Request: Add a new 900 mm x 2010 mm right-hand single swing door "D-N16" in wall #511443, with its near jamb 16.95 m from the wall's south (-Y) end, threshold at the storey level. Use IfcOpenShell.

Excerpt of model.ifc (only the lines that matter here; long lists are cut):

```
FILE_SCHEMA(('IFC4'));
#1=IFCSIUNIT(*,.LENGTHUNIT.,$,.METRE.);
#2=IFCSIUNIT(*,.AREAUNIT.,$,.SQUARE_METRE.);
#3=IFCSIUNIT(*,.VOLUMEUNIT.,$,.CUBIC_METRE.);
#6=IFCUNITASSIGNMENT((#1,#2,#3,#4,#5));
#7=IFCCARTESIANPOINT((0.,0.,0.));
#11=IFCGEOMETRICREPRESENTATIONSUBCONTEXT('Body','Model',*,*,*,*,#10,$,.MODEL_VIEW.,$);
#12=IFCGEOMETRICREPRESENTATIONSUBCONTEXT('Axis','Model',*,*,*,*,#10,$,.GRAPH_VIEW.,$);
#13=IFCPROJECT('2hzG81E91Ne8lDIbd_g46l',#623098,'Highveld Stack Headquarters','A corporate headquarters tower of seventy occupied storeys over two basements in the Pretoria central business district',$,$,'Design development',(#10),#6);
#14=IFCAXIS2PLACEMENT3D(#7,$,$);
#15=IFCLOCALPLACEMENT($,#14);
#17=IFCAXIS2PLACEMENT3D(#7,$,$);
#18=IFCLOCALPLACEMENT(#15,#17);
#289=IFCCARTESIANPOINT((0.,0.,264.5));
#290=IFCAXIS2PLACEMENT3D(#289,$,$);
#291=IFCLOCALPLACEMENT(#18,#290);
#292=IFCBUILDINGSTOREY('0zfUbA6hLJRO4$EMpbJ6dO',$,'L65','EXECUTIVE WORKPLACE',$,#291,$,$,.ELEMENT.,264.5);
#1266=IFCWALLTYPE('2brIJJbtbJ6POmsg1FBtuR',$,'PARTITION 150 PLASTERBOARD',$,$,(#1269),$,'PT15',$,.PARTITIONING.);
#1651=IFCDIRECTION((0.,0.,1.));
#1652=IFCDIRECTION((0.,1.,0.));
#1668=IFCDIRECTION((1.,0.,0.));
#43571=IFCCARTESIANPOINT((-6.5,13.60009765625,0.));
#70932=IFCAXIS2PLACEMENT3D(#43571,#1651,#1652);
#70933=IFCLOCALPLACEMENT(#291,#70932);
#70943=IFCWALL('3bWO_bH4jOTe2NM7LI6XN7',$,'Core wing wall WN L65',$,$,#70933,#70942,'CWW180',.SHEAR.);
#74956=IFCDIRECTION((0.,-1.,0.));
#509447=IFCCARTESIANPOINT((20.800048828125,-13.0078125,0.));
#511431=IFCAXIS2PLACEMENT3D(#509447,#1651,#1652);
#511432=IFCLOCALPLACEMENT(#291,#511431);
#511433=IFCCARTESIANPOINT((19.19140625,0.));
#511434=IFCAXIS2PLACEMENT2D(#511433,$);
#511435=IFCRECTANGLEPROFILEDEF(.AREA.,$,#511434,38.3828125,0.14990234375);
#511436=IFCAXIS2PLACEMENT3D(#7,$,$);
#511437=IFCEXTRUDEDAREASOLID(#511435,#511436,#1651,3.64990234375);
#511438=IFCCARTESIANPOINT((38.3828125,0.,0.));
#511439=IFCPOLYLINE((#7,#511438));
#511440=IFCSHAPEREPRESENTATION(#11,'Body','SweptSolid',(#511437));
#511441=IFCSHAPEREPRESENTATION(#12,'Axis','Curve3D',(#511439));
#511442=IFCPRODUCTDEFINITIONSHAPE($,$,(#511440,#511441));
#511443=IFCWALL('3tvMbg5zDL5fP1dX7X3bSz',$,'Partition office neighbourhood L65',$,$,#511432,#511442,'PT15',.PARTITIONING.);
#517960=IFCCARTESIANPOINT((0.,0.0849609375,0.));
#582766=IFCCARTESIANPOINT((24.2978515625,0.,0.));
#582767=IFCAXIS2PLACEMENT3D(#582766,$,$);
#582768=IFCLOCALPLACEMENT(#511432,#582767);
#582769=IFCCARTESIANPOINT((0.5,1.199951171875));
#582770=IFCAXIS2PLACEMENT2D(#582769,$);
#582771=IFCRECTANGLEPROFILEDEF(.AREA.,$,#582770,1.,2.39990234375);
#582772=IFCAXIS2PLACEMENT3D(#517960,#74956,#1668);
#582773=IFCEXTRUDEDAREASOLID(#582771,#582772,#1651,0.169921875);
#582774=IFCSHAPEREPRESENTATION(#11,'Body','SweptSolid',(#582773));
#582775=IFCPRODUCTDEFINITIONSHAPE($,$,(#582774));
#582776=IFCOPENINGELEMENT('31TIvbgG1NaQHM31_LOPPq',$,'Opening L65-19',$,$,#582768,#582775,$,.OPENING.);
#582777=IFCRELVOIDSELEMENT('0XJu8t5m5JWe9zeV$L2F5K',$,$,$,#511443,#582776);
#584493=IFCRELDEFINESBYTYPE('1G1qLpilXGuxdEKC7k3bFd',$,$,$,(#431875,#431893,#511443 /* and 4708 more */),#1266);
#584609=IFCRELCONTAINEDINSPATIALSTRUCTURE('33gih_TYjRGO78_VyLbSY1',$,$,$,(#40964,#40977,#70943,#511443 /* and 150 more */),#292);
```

```python
import numpy as np
import ifcopenshell
import ifcopenshell.api.feature
import ifcopenshell.api.geometry
import ifcopenshell.api.root
import ifcopenshell.api.spatial
import ifcopenshell.geom
import ifcopenshell.util.element
import ifcopenshell.util.placement
import ifcopenshell.util.representation
import ifcopenshell.util.shape
import ifcopenshell.util.unit

model = ifcopenshell.open("model.ifc")
unit_scale = ifcopenshell.util.unit.calculate_unit_scale(model)
settings = ifcopenshell.geom.settings()


def volume(element):
    """Net volume in cubic metres, openings subtracted."""
    shape = ifcopenshell.geom.create_shape(settings, element)
    return ifcopenshell.util.shape.get_volume(shape.geometry)


wall = model.by_guid("3tvMbg5zDL5fP1dX7X3bSz")
storey = ifcopenshell.util.element.get_container(wall, ifc_class="IfcBuildingStorey")
context = ifcopenshell.util.representation.get_context(model, "Model", "Body", "MODEL_VIEW")
before = volume(wall)

width, height, from_end, sill = 0.9, 2.01, 16.95, 0.0  # metres

# The wall runs along its own X axis, and the end named is its -X end.
wall_shape = ifcopenshell.geom.create_shape(settings, wall)
x, y, z = ifcopenshell.util.shape.get_vertices(wall_shape.geometry).T
start = x.min() + from_end
face, thickness = float(y.min()), float(y.max() - y.min())
wall_matrix = ifcopenshell.util.placement.get_local_placement(wall.ObjectPlacement)
level = ifcopenshell.util.placement.get_local_placement(storey.ObjectPlacement)[2, 3]


def in_wall(x, y):
    """Placement at x, y metres in the wall's axes, at sill height."""
    matrix = wall_matrix.copy()
    matrix[:, 3] = wall_matrix @ np.array([x / unit_scale, y / unit_scale, 0.0, 1.0])
    matrix[2, 3] = level + sill / unit_scale
    return matrix


# Opening: a box that overshoots both wall faces by 50 mm.
opening = ifcopenshell.api.root.create_entity(model, ifc_class="IfcOpeningElement", predefined_type="OPENING")
box = ifcopenshell.api.geometry.add_wall_representation(
    model, context=context, length=width, height=height, thickness=thickness + 0.1
)
ifcopenshell.api.geometry.assign_representation(model, product=opening, representation=box)
ifcopenshell.api.geometry.edit_object_placement(model, product=opening, matrix=in_wall(start, face - 0.05), is_si=False)
ifcopenshell.api.feature.add_feature(model, feature=opening, element=wall)

door = ifcopenshell.api.root.create_entity(model, ifc_class="IfcDoor", name="D-N16", predefined_type="DOOR")
door.OverallWidth, door.OverallHeight = width / unit_scale, height / unit_scale
door.OperationType = "SINGLE_SWING_RIGHT"
body = ifcopenshell.api.geometry.add_door_representation(
    model,
    context=context,
    overall_width=door.OverallWidth,
    overall_height=door.OverallHeight,
    operation_type="SINGLE_SWING_RIGHT",
    lining_properties={"LiningDepth": thickness / unit_scale, "ThresholdDepth": thickness / unit_scale},
)
ifcopenshell.api.geometry.assign_representation(model, product=door, representation=body)
ifcopenshell.api.spatial.assign_container(model, products=[door], relating_structure=storey)
ifcopenshell.api.feature.add_filling(model, opening=opening, element=door)

# The lining spans the wall, so the door starts at the wall face.
ifcopenshell.api.geometry.edit_object_placement(model, product=door, matrix=in_wall(start, face), is_si=False)

after = volume(wall)

print(f"wall volume {before:.3f} -> {after:.3f} m3")

model.write("model_edited.ifc")
```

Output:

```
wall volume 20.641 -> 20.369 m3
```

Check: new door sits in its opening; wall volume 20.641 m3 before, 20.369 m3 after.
